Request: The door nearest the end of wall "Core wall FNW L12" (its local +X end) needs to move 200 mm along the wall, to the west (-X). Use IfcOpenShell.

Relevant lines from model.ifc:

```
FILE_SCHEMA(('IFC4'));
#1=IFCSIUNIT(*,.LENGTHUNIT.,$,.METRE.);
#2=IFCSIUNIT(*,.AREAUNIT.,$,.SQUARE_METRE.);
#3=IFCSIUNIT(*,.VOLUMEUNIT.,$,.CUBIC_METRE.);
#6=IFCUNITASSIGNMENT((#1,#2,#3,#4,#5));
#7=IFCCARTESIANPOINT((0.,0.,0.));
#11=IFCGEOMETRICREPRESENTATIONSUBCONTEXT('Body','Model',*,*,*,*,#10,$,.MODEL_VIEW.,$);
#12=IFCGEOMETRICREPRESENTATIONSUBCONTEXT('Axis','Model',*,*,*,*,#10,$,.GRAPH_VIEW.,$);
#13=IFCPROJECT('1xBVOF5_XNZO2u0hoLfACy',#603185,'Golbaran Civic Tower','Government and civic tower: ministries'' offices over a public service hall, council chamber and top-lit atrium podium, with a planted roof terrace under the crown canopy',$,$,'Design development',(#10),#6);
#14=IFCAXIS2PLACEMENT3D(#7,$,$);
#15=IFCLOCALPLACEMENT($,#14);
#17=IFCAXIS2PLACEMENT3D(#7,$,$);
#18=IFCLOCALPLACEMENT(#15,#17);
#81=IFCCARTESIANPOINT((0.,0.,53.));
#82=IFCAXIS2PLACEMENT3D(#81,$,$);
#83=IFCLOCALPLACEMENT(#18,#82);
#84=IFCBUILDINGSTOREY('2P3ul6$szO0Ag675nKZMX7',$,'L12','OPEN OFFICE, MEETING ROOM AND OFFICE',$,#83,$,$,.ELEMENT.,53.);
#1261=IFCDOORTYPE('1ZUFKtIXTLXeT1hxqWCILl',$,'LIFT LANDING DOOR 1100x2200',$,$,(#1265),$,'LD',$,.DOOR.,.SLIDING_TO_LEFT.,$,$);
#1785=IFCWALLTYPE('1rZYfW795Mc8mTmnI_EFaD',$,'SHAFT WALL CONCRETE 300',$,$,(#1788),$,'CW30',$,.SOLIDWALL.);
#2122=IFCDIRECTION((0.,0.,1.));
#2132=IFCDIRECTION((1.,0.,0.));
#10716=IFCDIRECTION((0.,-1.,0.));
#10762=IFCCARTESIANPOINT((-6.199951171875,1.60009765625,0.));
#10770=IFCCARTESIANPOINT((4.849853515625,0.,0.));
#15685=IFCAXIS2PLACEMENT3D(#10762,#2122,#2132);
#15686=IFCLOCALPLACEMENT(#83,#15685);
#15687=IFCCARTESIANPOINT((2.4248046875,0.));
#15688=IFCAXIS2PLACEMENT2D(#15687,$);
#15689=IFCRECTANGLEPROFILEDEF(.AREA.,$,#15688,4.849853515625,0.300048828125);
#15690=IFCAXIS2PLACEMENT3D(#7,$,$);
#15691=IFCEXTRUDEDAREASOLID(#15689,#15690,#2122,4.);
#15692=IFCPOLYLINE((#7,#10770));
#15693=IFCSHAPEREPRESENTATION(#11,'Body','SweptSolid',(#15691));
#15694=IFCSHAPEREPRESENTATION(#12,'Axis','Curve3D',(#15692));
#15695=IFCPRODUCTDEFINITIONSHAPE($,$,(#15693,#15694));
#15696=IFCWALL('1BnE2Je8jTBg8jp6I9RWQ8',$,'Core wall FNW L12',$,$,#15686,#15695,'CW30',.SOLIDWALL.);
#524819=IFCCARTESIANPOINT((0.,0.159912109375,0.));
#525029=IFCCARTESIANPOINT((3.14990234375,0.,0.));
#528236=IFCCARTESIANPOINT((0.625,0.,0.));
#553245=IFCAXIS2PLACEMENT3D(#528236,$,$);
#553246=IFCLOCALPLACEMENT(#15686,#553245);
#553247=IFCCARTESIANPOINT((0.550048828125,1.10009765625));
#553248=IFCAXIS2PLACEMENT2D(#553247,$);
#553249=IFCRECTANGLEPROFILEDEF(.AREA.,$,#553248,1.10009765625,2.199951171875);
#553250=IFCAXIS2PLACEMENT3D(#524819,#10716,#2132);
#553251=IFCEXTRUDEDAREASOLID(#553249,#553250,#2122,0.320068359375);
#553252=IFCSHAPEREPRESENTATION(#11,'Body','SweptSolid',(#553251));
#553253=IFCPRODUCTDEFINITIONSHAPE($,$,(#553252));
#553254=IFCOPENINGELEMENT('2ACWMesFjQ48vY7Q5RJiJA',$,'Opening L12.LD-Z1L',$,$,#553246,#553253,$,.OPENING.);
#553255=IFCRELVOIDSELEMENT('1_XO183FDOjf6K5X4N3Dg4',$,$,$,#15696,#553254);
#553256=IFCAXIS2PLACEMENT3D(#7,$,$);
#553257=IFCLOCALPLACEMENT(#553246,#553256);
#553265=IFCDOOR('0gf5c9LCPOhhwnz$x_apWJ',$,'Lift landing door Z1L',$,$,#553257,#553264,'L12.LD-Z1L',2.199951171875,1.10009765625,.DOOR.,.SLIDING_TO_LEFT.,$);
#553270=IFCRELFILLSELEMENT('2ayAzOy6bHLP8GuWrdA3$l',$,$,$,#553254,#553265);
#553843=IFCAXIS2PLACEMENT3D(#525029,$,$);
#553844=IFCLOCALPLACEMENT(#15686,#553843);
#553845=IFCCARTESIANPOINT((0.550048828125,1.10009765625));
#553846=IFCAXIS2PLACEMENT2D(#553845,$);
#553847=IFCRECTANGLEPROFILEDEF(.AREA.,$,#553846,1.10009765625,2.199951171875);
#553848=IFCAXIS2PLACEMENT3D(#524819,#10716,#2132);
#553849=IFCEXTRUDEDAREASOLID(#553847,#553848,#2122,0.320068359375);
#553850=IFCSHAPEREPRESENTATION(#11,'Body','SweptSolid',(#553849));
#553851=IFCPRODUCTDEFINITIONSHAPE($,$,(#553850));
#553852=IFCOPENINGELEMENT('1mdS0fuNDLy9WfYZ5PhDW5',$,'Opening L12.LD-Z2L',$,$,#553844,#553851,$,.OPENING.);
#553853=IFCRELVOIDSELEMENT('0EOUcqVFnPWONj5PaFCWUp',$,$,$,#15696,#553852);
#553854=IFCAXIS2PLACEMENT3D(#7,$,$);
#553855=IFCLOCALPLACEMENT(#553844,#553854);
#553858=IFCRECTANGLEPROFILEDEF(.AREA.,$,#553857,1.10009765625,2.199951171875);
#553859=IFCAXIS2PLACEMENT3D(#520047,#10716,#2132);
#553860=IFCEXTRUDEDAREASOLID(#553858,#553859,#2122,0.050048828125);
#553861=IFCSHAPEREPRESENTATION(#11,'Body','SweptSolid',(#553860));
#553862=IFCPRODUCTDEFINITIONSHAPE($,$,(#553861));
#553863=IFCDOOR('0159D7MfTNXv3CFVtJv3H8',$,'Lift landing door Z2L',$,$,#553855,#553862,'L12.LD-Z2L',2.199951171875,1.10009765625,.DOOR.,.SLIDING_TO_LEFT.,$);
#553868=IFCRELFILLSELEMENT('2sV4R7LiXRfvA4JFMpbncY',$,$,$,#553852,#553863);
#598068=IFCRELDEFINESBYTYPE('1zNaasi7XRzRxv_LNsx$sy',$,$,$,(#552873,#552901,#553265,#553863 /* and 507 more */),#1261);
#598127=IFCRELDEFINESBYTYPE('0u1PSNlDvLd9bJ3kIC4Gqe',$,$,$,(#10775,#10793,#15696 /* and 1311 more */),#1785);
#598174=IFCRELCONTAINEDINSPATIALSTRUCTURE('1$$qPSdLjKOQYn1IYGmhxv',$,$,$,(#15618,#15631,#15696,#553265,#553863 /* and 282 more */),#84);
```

```python
import ifcopenshell
import ifcopenshell.api.geometry
import ifcopenshell.util.placement

model = ifcopenshell.open("model.ifc")

door = model.by_id(553863)
opening = door.FillsVoids[0].RelatingOpeningElement
wall = opening.VoidsElements[0].RelatingBuildingElement

wall_matrix = ifcopenshell.util.placement.get_local_placement(wall.ObjectPlacement)
shift = wall_matrix[:3, 0] * -0.2
before = ifcopenshell.util.placement.get_local_placement(door.ObjectPlacement)[:3, 3].copy()

# The door is placed relative to its opening, so it follows when the opening moves.
matrix = ifcopenshell.util.placement.get_local_placement(opening.ObjectPlacement)
matrix[:3, 3] += shift
ifcopenshell.api.geometry.edit_object_placement(
    model, product=opening, matrix=matrix, is_si=False, should_transform_children=True
)

after = ifcopenshell.util.placement.get_local_placement(door.ObjectPlacement)[:3, 3]
print("door moved by", (after - before).round(3) + 0.0)

model.write("model-out.ifc")
```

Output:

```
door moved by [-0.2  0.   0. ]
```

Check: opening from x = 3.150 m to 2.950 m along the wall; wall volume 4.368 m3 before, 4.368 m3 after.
